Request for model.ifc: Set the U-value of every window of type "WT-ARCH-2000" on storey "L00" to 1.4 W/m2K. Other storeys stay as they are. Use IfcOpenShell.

First a look at what the model holds.

```python
import ifcopenshell
import ifcopenshell.util.element

model = ifcopenshell.open("model.ifc")
print(model.schema)
storey = next(s for s in model.by_type("IfcBuildingStorey") if s.Name == "L00")
windows = [e for e in ifcopenshell.util.element.get_decomposition(storey) if e.is_a("IfcWindow")]
seen = {}
for e in windows:
    element_type = ifcopenshell.util.element.get_type(e)
    key = (element_type.Name if element_type != e and element_type else None, ifcopenshell.util.element.get_pset(e, "Pset_WindowCommon", "ThermalTransmittance"))
    seen[key] = seen.get(key, 0) + 1
for (name, value), count in sorted(seen.items(), key=str):
    print(count, "x", name, "|", value)
```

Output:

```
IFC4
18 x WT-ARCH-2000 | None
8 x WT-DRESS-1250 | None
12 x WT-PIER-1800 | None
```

```python
import ifcopenshell
import ifcopenshell.api.pset
import ifcopenshell.util.element

model = ifcopenshell.open("model.ifc")

storey = next(s for s in model.by_type("IfcBuildingStorey") if s.Name == "L00")
windows = [e for e in ifcopenshell.util.element.get_decomposition(storey) if e.is_a("IfcWindow")]

count = 0
for e in windows:
    element_type = ifcopenshell.util.element.get_type(e)
    if element_type in (None, e) or element_type.Name != "WT-ARCH-2000":
        continue
    # add_pset returns the element's existing set when there is one.
    pset = ifcopenshell.api.pset.add_pset(model, product=e, name="Pset_WindowCommon")
    ifcopenshell.api.pset.edit_pset(model, pset=pset, properties={"ThermalTransmittance": 1.4})
    count += 1

print(count, "windows updated")

model.write("model_rev.ifc")
```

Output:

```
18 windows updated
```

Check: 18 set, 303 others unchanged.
